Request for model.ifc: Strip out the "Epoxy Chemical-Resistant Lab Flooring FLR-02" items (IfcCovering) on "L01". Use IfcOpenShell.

First a look at what the model holds.

```python
import ifcopenshell
import ifcopenshell.util.element

model = ifcopenshell.open("model.ifc")
print(model.schema)
storey = next(s for s in model.by_type("IfcBuildingStorey") if s.Name == "L01")
coverings = [e for e in ifcopenshell.util.element.get_decomposition(storey) if e.is_a("IfcCovering")]
seen = {}
for e in coverings:
    element_type = ifcopenshell.util.element.get_type(e)
    name = element_type.Name if element_type not in (None, e) else None
    seen[name] = seen.get(name, 0) + 1
for name, count in sorted(seen.items(), key=str):
    print(count, "x", name)
```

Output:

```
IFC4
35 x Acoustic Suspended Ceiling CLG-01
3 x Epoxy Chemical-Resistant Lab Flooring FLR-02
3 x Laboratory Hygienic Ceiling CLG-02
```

```python
import ifcopenshell
import ifcopenshell.api.root
import ifcopenshell.util.element

model = ifcopenshell.open("model.ifc")

storey = next(s for s in model.by_type("IfcBuildingStorey") if s.Name == "L01")
coverings = [e for e in ifcopenshell.util.element.get_decomposition(storey) if e.is_a("IfcCovering")]
targets = [e for e in coverings if (t := ifcopenshell.util.element.get_type(e)) not in (None, e) and t.Name == "Epoxy Chemical-Resistant Lab Flooring FLR-02"]

for e in targets:
    ifcopenshell.api.root.remove_product(model, product=e)
print(len(targets), "removed")

model.write("model_rev.ifc")
```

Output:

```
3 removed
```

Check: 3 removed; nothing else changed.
